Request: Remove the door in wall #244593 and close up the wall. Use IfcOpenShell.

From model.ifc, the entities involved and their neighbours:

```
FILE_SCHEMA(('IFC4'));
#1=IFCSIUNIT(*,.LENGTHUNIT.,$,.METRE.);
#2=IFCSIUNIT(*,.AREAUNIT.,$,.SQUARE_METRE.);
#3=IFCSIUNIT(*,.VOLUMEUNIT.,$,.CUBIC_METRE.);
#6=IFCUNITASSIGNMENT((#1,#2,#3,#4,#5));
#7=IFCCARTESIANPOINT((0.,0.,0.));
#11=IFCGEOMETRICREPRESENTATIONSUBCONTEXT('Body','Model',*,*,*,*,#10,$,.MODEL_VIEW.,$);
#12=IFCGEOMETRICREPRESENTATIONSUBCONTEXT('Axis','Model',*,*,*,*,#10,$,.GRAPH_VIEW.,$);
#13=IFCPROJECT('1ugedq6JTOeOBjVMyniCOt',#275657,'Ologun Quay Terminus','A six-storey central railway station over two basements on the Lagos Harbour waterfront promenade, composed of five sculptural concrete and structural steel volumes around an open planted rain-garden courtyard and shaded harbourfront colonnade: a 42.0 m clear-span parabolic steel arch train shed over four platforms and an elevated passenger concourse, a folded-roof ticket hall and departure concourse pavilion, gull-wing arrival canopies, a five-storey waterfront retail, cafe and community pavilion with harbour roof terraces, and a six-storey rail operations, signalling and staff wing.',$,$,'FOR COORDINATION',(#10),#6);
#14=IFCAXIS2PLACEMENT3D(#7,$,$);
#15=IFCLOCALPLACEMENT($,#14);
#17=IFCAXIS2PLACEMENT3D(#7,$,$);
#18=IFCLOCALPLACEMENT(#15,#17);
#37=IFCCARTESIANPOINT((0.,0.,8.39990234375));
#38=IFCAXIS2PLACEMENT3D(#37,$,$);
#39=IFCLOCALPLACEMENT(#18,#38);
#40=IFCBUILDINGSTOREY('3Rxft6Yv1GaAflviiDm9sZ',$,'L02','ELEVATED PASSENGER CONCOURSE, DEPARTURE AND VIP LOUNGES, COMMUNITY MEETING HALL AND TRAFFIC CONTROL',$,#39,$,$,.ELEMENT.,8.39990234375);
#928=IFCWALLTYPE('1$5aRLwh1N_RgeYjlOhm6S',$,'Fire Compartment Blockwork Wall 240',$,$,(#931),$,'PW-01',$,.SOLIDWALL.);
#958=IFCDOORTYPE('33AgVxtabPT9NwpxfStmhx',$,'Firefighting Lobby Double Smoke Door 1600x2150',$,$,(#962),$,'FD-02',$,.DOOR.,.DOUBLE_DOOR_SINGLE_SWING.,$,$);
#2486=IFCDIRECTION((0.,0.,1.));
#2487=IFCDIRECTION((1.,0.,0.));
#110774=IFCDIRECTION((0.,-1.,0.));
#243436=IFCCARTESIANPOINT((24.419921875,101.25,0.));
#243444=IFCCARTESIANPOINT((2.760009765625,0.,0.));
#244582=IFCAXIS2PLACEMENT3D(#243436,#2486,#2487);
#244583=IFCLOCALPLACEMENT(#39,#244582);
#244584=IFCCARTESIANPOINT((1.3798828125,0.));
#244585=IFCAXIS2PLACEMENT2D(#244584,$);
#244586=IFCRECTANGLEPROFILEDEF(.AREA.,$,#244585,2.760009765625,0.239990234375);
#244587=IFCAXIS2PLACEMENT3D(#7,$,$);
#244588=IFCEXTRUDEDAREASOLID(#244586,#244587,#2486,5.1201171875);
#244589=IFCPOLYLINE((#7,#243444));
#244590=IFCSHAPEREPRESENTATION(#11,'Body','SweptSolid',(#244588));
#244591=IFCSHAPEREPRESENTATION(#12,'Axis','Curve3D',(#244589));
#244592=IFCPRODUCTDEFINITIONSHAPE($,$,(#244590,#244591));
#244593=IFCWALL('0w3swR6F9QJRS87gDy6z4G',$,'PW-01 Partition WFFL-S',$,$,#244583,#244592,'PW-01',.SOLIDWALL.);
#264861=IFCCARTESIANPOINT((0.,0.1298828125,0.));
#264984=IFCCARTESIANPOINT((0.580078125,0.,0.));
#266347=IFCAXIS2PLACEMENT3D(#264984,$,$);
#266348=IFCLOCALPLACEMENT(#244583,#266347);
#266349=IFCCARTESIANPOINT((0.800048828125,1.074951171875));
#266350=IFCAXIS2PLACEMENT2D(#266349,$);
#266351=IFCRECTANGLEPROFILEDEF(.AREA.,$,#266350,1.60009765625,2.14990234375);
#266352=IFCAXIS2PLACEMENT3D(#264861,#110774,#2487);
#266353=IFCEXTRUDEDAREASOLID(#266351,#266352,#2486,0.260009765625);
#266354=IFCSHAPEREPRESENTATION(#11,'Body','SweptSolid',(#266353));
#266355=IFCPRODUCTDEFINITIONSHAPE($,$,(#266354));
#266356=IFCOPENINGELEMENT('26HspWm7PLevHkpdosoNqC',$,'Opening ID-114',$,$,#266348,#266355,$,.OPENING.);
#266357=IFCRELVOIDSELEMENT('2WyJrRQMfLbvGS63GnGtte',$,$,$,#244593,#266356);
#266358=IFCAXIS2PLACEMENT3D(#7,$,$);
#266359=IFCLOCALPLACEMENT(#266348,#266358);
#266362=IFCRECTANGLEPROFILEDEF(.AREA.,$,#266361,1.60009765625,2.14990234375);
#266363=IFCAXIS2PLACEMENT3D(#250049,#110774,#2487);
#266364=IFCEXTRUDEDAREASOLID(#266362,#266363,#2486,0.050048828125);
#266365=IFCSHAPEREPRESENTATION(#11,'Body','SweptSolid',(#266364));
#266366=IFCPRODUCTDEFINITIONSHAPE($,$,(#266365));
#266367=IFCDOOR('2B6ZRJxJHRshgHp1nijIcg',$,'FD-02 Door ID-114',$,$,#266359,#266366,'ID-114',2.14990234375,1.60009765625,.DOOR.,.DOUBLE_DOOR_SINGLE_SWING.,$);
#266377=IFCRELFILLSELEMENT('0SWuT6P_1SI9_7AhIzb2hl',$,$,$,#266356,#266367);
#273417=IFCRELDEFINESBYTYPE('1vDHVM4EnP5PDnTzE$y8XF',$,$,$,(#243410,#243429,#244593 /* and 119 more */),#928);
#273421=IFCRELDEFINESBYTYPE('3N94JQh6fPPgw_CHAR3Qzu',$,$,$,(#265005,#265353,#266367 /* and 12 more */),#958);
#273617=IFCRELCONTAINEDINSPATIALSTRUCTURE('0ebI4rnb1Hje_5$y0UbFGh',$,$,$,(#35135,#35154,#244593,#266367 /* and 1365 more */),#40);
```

```python
import ifcopenshell
import ifcopenshell.api.feature
import ifcopenshell.api.root
import ifcopenshell.geom
import ifcopenshell.util.shape

model = ifcopenshell.open("model.ifc")
settings = ifcopenshell.geom.settings()


def volume(element):
    """Net volume in cubic metres, openings subtracted."""
    shape = ifcopenshell.geom.create_shape(settings, element)
    return ifcopenshell.util.shape.get_volume(shape.geometry)


door = model.by_guid("2B6ZRJxJHRshgHp1nijIcg")
opening = door.FillsVoids[0].RelatingOpeningElement
wall = opening.VoidsElements[0].RelatingBuildingElement
before = volume(wall)

ifcopenshell.api.root.remove_product(model, product=door)
ifcopenshell.api.feature.remove_feature(model, feature=opening)

after = volume(wall)

print(f"wall volume {before:.3f} -> {after:.3f} m3")

model.write("model_updated.ifc")
```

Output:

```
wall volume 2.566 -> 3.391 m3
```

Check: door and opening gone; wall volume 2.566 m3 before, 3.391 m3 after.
